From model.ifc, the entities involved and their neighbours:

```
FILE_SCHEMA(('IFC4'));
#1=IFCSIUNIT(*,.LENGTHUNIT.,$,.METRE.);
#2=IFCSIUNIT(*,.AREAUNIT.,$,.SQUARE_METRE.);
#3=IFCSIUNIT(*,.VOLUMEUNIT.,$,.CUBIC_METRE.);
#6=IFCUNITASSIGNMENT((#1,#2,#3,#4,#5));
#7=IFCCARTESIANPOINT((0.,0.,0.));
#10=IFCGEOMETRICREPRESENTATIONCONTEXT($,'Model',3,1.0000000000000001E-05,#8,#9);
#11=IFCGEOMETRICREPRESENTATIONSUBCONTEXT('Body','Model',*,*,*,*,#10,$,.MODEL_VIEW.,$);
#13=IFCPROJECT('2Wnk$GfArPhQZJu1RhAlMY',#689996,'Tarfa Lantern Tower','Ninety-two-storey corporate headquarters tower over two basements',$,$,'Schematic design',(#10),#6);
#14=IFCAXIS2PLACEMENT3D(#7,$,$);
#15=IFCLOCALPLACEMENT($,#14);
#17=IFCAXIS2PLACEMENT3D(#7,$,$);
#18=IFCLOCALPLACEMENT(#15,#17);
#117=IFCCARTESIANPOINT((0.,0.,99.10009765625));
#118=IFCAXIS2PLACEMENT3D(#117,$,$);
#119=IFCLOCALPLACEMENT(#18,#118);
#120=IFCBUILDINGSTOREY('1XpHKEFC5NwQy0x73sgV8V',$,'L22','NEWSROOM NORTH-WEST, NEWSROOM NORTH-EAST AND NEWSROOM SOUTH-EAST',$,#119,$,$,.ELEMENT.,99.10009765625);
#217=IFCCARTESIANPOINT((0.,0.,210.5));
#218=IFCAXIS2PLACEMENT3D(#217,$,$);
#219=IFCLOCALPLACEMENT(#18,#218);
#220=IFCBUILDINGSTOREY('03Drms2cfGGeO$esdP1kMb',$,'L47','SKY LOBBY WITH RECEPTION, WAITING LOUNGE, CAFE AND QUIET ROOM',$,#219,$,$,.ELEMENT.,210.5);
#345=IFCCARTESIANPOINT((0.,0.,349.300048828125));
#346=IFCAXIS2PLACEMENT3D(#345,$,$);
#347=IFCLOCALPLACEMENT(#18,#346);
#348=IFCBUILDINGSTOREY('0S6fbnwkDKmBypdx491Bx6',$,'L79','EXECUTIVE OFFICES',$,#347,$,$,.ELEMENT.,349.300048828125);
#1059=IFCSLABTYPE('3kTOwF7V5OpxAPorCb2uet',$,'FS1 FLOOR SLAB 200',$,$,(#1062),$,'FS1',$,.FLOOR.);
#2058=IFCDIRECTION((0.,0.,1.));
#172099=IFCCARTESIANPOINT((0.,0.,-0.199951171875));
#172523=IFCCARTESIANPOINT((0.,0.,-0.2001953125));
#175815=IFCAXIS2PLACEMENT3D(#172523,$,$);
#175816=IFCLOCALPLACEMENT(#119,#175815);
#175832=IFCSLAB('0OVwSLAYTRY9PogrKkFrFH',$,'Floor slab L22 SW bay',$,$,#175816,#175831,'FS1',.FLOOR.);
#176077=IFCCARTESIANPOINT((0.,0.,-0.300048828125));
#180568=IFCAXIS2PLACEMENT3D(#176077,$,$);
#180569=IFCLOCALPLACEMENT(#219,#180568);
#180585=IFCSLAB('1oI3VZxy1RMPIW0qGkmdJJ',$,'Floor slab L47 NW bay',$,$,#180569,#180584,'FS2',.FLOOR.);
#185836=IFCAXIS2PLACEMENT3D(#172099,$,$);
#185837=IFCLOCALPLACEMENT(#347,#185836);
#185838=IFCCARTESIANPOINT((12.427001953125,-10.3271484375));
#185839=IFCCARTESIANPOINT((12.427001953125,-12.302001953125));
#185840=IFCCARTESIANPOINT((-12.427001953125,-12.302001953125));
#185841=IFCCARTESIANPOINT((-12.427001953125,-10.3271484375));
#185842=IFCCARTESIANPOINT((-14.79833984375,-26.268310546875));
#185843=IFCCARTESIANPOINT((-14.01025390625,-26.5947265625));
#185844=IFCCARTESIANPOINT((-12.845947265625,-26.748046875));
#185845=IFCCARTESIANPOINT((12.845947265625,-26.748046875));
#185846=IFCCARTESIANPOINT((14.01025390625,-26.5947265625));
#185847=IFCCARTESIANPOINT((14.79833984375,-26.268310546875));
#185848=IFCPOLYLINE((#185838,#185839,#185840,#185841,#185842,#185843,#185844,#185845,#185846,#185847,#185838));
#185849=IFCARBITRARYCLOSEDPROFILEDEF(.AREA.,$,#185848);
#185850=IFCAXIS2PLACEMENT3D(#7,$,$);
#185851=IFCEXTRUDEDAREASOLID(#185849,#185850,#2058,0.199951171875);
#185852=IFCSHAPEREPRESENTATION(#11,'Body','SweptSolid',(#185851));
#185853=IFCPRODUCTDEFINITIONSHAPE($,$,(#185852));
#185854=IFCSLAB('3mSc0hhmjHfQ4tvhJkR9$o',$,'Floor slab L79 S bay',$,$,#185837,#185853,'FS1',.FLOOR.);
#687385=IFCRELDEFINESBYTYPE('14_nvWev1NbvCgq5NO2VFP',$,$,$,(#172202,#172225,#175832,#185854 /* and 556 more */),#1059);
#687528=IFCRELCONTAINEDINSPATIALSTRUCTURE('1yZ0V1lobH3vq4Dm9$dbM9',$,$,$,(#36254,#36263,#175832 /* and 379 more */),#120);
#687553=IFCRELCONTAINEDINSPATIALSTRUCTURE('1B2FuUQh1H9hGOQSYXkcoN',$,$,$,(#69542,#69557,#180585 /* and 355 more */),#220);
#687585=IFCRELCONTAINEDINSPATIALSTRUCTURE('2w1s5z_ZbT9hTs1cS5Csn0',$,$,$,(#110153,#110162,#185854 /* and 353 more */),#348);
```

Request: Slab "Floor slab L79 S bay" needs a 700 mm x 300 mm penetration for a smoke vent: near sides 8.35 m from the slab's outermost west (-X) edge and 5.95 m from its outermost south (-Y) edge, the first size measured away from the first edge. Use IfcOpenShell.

```python
import numpy as np
import ifcopenshell
import ifcopenshell.api.feature
import ifcopenshell.api.geometry
import ifcopenshell.api.root
import ifcopenshell.geom
import ifcopenshell.util.placement
import ifcopenshell.util.representation
import ifcopenshell.util.shape
import ifcopenshell.util.unit

model = ifcopenshell.open("model.ifc")
unit_scale = ifcopenshell.util.unit.calculate_unit_scale(model)
settings = ifcopenshell.geom.settings()


def volume(element):
    """Net volume in cubic metres, openings subtracted."""
    shape = ifcopenshell.geom.create_shape(settings, element)
    return ifcopenshell.util.shape.get_volume(shape.geometry)


slab = model.by_id(185854)
before = volume(slab)

# Extent in the slab's own axes, in metres. The edges named are its -X and -Y sides.
slab_shape = ifcopenshell.geom.create_shape(settings, slab)
vertices = ifcopenshell.util.shape.get_vertices(slab_shape.geometry)
x_min, y_min, bottom = vertices.min(axis=0)
top = vertices[:, 2].max()

opening = ifcopenshell.api.root.create_entity(model, ifc_class="IfcOpeningElement", name="Smoke vent opening", predefined_type="OPENING")
context = ifcopenshell.util.representation.get_context(model, "Model", "Body", "MODEL_VIEW")
width, depth = 0.7, 0.3
outline = [(0.0, 0.0), (width, 0.0), (width, depth), (0.0, depth), (0.0, 0.0)]
# Overshoot both faces by 50 mm so the cut is clean.
shape = ifcopenshell.api.geometry.add_slab_representation(
    model, context=context, depth=top - bottom + 0.1, polyline=outline
)
ifcopenshell.api.geometry.assign_representation(model, product=opening, representation=shape)

matrix = ifcopenshell.util.placement.get_local_placement(slab.ObjectPlacement)
matrix[:, 3] = matrix @ np.append(np.array([x_min + 8.35, y_min + 5.95, bottom - 0.05]) / unit_scale, 1.0)
ifcopenshell.api.geometry.edit_object_placement(model, product=opening, matrix=matrix, is_si=False)
ifcopenshell.api.feature.add_feature(model, feature=opening, element=slab)

after = volume(slab)

print(f"slab volume {before:.3f} -> {after:.3f} m3")

model.write("model_rev.ifc")
```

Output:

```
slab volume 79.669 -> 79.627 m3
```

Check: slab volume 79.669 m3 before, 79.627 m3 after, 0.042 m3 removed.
